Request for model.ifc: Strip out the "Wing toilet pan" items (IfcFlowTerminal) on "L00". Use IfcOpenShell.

First a look at what the model holds.

```python
import ifcopenshell
import ifcopenshell.util.element

model = ifcopenshell.open("model.ifc")
print(model.schema)
storey = next(s for s in model.by_type("IfcBuildingStorey") if s.Name == "L00")
terminals = [e for e in ifcopenshell.util.element.get_decomposition(storey) if e.is_a("IfcFlowTerminal")]
seen = {}
for e in terminals:
    element_type = ifcopenshell.util.element.get_type(e)
    name = element_type.Name if element_type not in (None, e) else None
    seen[name] = seen.get(name, 0) + 1
for name, count in sorted(seen.items(), key=str):
    print(count, "x", name)
```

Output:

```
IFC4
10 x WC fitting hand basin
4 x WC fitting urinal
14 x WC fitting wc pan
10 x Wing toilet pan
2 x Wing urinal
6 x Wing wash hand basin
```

```python
import ifcopenshell
import ifcopenshell.api.root
import ifcopenshell.util.element

model = ifcopenshell.open("model.ifc")

storey = next(s for s in model.by_type("IfcBuildingStorey") if s.Name == "L00")
terminals = [e for e in ifcopenshell.util.element.get_decomposition(storey) if e.is_a("IfcFlowTerminal")]
targets = [e for e in terminals if (t := ifcopenshell.util.element.get_type(e)) not in (None, e) and t.Name == "Wing toilet pan"]

for e in targets:
    ifcopenshell.api.root.remove_product(model, product=e)
print(len(targets), "removed")

model.write("model_rev.ifc")
```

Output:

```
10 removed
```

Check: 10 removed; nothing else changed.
